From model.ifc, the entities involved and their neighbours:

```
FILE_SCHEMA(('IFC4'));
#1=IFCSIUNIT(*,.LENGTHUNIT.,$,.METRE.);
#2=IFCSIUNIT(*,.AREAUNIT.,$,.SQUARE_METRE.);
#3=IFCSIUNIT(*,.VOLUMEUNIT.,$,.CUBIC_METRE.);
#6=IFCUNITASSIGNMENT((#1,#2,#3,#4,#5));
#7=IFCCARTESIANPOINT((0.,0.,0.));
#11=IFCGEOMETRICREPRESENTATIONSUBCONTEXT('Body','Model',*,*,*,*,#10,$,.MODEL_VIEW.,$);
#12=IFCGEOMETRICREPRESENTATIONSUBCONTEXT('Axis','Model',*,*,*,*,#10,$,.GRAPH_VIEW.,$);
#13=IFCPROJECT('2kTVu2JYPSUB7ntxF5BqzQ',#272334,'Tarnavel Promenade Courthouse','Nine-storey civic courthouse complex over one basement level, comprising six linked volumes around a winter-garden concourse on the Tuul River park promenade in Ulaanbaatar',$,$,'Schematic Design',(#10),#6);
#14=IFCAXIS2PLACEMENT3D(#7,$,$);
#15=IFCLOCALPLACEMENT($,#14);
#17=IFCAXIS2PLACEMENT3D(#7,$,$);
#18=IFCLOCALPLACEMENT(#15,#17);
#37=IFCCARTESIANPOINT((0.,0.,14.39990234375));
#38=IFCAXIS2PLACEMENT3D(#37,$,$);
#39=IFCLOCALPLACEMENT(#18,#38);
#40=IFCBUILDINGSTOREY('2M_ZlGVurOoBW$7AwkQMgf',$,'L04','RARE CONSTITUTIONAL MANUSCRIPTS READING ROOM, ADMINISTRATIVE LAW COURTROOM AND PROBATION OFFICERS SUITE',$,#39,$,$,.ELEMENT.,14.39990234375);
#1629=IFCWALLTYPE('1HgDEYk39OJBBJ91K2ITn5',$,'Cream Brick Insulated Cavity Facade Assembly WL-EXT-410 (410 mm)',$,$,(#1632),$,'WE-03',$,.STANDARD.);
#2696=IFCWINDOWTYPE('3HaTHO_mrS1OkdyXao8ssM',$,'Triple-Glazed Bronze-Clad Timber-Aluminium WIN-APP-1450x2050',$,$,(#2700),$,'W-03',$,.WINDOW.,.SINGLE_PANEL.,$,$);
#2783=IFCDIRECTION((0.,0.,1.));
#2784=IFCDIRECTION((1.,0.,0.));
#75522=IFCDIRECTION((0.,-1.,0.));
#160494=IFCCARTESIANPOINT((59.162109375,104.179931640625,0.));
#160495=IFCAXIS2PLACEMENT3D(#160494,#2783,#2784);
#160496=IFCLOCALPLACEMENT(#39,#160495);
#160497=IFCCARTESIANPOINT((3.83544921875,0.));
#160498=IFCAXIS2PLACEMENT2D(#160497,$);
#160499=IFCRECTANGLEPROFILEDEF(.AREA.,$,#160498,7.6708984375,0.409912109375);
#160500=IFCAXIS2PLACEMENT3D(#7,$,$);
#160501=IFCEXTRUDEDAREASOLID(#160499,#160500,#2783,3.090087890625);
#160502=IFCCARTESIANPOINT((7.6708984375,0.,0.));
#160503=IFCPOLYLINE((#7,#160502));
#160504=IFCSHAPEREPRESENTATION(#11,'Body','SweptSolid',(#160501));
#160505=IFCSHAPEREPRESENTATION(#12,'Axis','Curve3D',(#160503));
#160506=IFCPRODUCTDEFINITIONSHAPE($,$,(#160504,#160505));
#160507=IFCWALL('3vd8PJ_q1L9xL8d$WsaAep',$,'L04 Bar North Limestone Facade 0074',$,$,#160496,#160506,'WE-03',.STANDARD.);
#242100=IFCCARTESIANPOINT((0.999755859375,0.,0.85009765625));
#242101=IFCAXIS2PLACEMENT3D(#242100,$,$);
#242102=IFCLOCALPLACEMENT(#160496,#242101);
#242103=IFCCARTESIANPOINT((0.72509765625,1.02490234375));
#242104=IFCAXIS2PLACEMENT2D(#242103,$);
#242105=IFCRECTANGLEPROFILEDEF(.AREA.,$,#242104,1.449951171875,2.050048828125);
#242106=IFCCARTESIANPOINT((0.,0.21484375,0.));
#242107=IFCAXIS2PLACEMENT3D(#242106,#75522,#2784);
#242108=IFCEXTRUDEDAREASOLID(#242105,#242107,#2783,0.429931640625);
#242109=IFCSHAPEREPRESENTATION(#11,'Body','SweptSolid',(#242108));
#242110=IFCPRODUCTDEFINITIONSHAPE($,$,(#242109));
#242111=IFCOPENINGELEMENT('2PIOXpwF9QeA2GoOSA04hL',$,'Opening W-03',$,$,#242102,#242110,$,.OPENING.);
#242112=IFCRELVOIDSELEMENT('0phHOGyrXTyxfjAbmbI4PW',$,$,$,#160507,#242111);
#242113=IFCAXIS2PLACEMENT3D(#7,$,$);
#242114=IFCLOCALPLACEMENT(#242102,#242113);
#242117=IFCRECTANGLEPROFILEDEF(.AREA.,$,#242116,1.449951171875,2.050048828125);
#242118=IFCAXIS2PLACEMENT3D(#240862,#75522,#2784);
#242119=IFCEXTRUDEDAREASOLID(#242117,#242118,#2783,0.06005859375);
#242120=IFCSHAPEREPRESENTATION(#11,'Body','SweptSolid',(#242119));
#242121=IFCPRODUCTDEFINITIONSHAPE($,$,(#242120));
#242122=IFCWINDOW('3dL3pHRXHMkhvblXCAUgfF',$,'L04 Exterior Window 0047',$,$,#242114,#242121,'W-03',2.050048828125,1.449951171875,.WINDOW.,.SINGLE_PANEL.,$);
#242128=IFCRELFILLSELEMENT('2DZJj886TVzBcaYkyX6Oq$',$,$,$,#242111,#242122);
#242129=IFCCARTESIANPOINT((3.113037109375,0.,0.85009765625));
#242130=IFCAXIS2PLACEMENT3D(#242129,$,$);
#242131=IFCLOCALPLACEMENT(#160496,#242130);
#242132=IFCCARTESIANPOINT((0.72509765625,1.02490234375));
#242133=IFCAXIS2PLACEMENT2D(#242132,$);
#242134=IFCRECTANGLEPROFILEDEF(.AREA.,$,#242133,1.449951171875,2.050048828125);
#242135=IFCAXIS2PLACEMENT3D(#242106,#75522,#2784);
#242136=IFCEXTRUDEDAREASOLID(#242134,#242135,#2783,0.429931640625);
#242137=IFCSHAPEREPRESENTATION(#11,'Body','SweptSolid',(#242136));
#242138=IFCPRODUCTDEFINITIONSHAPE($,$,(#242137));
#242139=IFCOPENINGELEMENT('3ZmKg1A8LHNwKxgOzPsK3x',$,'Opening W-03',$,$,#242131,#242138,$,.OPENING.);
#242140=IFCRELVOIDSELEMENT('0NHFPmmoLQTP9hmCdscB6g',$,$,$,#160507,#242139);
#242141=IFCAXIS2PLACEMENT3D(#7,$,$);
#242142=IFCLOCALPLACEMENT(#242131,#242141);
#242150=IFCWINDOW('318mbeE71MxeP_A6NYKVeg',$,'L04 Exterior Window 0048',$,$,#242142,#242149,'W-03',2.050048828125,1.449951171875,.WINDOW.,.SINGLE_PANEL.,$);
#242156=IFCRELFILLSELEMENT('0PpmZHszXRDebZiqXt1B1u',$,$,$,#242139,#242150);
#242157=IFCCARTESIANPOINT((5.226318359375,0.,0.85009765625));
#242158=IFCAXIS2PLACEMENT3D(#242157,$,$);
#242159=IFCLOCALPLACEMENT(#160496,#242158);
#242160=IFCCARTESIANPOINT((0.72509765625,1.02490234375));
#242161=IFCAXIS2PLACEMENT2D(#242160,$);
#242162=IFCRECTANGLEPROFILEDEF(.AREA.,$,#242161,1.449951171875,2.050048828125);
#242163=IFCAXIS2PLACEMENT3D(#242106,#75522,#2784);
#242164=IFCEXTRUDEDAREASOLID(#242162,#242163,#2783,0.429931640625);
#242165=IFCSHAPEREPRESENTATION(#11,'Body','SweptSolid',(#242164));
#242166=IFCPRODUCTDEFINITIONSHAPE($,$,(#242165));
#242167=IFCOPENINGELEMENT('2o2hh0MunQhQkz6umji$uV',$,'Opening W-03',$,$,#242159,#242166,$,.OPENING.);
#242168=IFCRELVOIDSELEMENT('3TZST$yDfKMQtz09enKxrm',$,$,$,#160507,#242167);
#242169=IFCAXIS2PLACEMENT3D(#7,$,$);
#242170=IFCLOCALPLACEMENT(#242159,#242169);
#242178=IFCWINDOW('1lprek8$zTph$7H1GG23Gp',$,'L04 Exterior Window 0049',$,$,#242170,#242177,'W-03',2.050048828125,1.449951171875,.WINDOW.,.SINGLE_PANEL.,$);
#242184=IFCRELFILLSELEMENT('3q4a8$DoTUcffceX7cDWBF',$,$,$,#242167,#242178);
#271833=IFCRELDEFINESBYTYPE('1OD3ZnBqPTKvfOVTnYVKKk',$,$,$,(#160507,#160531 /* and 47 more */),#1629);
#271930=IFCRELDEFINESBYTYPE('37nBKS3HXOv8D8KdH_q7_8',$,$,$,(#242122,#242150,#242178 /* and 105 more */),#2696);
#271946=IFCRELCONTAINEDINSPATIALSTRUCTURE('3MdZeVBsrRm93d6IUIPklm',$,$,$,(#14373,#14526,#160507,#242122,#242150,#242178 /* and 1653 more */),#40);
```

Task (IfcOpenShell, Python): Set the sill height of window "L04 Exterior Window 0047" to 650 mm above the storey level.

```python
import numpy as np
import ifcopenshell
import ifcopenshell.api.geometry
import ifcopenshell.geom
import ifcopenshell.util.element
import ifcopenshell.util.placement
import ifcopenshell.util.shape
import ifcopenshell.util.unit

model = ifcopenshell.open("model.ifc")
unit_scale = ifcopenshell.util.unit.calculate_unit_scale(model)

window = model.by_id(242122)
opening = window.FillsVoids[0].RelatingOpeningElement
storey = ifcopenshell.util.element.get_container(window, ifc_class="IfcBuildingStorey")
level = ifcopenshell.util.placement.get_local_placement(storey.ObjectPlacement)[2, 3]

# The opening's origin need not be at the sill, so measure its lowest point.
shape = ifcopenshell.geom.create_shape(ifcopenshell.geom.settings(), opening)
bottom = ifcopenshell.util.shape.get_shape_bottom_elevation(shape, shape.geometry) / unit_scale
dz = level + 0.65 - bottom

shift = np.array([0.0, 0.0, dz])
# The window is placed relative to its opening, so it follows when the opening moves.
matrix = ifcopenshell.util.placement.get_local_placement(opening.ObjectPlacement)
matrix[:3, 3] += shift
ifcopenshell.api.geometry.edit_object_placement(
    model, product=opening, matrix=matrix, is_si=False, should_transform_children=True
)

print(f"moved by {dz * unit_scale:+.3f} m")

model.write("model_rev.ifc")
```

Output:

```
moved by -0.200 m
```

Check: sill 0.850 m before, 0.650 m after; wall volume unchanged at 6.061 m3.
